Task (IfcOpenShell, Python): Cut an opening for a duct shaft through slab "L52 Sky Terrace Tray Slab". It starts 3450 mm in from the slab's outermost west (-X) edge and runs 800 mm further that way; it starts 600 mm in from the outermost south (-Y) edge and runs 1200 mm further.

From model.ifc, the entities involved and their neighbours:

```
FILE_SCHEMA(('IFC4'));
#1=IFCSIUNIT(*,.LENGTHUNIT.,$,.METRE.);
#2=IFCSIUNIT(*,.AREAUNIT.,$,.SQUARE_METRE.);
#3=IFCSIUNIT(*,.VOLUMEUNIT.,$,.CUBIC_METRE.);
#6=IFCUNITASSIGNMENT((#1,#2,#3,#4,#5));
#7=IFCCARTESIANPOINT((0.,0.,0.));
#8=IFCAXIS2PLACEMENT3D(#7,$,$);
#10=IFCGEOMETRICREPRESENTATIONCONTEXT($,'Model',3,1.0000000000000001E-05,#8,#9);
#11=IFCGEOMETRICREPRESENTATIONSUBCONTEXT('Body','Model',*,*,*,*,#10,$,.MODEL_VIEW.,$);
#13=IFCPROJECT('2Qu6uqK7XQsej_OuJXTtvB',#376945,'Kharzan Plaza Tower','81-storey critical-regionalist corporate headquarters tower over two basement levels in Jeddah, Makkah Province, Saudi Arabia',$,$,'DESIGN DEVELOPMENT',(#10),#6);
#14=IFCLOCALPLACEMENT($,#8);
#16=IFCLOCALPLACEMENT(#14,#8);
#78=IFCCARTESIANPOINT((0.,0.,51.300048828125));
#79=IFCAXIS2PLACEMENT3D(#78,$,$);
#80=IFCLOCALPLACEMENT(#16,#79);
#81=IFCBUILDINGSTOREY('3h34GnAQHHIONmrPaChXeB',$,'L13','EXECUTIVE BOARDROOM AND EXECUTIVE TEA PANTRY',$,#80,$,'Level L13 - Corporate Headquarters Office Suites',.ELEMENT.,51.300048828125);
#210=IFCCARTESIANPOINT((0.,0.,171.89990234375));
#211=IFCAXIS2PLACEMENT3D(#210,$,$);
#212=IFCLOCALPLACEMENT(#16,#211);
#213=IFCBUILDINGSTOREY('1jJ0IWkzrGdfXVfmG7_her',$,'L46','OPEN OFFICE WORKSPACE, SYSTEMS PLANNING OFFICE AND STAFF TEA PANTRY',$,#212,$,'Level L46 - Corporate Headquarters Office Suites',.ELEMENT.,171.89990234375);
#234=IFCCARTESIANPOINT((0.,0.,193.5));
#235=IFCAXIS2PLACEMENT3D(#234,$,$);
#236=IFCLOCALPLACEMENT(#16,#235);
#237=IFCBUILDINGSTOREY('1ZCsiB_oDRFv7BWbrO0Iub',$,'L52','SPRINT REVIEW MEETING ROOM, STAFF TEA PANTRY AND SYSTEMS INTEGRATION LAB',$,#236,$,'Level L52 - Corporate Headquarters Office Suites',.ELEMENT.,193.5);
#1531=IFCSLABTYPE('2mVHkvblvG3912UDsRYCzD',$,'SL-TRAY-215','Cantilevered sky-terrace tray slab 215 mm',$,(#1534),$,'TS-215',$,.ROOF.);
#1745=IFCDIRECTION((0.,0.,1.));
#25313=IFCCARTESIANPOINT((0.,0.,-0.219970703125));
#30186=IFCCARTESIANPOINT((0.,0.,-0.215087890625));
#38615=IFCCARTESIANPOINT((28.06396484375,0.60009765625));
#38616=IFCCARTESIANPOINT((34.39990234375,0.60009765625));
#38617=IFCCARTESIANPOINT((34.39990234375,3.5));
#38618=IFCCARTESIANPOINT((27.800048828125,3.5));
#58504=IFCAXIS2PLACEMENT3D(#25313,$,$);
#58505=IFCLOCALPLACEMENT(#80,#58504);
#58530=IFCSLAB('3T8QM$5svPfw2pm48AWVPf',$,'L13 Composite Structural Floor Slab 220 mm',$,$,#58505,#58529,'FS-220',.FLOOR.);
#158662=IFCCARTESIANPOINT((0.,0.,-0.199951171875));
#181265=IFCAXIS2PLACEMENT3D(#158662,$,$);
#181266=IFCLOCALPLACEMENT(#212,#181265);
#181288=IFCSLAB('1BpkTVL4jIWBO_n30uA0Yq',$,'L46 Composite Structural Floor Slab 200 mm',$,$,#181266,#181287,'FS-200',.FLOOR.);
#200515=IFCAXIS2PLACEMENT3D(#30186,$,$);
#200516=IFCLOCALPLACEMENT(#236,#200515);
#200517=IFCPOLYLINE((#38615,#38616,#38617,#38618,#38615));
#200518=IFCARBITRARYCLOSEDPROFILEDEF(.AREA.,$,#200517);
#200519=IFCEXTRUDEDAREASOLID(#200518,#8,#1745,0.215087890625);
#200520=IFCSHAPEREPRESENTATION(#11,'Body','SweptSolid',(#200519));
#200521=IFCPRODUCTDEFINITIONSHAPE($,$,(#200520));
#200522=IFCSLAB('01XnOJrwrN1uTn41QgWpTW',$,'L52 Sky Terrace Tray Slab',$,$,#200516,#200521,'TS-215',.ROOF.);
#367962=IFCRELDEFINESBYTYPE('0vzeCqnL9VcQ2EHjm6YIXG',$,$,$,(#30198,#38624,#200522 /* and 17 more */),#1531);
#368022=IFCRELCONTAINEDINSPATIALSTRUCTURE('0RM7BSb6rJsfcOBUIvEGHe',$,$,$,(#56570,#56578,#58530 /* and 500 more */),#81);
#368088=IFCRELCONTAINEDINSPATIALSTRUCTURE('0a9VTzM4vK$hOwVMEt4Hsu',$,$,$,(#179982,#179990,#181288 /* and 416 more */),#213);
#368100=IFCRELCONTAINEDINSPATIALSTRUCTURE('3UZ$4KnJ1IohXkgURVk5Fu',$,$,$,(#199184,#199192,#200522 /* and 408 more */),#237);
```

```python
import numpy as np
import ifcopenshell
import ifcopenshell.api.feature
import ifcopenshell.api.geometry
import ifcopenshell.api.root
import ifcopenshell.geom
import ifcopenshell.util.placement
import ifcopenshell.util.representation
import ifcopenshell.util.shape
import ifcopenshell.util.unit

model = ifcopenshell.open("model.ifc")
unit_scale = ifcopenshell.util.unit.calculate_unit_scale(model)
settings = ifcopenshell.geom.settings()


def volume(element):
    """Net volume in cubic metres, openings subtracted."""
    shape = ifcopenshell.geom.create_shape(settings, element)
    return ifcopenshell.util.shape.get_volume(shape.geometry)


slab = model.by_id(200522)
before = volume(slab)

# Extent in the slab's own axes, in metres. The edges named are its -X and -Y sides.
slab_shape = ifcopenshell.geom.create_shape(settings, slab)
vertices = ifcopenshell.util.shape.get_vertices(slab_shape.geometry)
x_min, y_min, bottom = vertices.min(axis=0)
top = vertices[:, 2].max()

opening = ifcopenshell.api.root.create_entity(model, ifc_class="IfcOpeningElement", name="Duct shaft opening", predefined_type="OPENING")
context = ifcopenshell.util.representation.get_context(model, "Model", "Body", "MODEL_VIEW")
width, depth = 0.8, 1.2
outline = [(0.0, 0.0), (width, 0.0), (width, depth), (0.0, depth), (0.0, 0.0)]
# Overshoot both faces by 50 mm so the cut is clean.
shape = ifcopenshell.api.geometry.add_slab_representation(
    model, context=context, depth=top - bottom + 0.1, polyline=outline
)
ifcopenshell.api.geometry.assign_representation(model, product=opening, representation=shape)

matrix = ifcopenshell.util.placement.get_local_placement(slab.ObjectPlacement)
matrix[:, 3] = matrix @ np.append(np.array([x_min + 3.45, y_min + 0.6, bottom - 0.05]) / unit_scale, 1.0)
ifcopenshell.api.geometry.edit_object_placement(model, product=opening, matrix=matrix, is_si=False)
ifcopenshell.api.feature.add_feature(model, feature=opening, element=slab)

after = volume(slab)

print(f"slab volume {before:.3f} -> {after:.3f} m3")

model.write("model_rev.ifc")
```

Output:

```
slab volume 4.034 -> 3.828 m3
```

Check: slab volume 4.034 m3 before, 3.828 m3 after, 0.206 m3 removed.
